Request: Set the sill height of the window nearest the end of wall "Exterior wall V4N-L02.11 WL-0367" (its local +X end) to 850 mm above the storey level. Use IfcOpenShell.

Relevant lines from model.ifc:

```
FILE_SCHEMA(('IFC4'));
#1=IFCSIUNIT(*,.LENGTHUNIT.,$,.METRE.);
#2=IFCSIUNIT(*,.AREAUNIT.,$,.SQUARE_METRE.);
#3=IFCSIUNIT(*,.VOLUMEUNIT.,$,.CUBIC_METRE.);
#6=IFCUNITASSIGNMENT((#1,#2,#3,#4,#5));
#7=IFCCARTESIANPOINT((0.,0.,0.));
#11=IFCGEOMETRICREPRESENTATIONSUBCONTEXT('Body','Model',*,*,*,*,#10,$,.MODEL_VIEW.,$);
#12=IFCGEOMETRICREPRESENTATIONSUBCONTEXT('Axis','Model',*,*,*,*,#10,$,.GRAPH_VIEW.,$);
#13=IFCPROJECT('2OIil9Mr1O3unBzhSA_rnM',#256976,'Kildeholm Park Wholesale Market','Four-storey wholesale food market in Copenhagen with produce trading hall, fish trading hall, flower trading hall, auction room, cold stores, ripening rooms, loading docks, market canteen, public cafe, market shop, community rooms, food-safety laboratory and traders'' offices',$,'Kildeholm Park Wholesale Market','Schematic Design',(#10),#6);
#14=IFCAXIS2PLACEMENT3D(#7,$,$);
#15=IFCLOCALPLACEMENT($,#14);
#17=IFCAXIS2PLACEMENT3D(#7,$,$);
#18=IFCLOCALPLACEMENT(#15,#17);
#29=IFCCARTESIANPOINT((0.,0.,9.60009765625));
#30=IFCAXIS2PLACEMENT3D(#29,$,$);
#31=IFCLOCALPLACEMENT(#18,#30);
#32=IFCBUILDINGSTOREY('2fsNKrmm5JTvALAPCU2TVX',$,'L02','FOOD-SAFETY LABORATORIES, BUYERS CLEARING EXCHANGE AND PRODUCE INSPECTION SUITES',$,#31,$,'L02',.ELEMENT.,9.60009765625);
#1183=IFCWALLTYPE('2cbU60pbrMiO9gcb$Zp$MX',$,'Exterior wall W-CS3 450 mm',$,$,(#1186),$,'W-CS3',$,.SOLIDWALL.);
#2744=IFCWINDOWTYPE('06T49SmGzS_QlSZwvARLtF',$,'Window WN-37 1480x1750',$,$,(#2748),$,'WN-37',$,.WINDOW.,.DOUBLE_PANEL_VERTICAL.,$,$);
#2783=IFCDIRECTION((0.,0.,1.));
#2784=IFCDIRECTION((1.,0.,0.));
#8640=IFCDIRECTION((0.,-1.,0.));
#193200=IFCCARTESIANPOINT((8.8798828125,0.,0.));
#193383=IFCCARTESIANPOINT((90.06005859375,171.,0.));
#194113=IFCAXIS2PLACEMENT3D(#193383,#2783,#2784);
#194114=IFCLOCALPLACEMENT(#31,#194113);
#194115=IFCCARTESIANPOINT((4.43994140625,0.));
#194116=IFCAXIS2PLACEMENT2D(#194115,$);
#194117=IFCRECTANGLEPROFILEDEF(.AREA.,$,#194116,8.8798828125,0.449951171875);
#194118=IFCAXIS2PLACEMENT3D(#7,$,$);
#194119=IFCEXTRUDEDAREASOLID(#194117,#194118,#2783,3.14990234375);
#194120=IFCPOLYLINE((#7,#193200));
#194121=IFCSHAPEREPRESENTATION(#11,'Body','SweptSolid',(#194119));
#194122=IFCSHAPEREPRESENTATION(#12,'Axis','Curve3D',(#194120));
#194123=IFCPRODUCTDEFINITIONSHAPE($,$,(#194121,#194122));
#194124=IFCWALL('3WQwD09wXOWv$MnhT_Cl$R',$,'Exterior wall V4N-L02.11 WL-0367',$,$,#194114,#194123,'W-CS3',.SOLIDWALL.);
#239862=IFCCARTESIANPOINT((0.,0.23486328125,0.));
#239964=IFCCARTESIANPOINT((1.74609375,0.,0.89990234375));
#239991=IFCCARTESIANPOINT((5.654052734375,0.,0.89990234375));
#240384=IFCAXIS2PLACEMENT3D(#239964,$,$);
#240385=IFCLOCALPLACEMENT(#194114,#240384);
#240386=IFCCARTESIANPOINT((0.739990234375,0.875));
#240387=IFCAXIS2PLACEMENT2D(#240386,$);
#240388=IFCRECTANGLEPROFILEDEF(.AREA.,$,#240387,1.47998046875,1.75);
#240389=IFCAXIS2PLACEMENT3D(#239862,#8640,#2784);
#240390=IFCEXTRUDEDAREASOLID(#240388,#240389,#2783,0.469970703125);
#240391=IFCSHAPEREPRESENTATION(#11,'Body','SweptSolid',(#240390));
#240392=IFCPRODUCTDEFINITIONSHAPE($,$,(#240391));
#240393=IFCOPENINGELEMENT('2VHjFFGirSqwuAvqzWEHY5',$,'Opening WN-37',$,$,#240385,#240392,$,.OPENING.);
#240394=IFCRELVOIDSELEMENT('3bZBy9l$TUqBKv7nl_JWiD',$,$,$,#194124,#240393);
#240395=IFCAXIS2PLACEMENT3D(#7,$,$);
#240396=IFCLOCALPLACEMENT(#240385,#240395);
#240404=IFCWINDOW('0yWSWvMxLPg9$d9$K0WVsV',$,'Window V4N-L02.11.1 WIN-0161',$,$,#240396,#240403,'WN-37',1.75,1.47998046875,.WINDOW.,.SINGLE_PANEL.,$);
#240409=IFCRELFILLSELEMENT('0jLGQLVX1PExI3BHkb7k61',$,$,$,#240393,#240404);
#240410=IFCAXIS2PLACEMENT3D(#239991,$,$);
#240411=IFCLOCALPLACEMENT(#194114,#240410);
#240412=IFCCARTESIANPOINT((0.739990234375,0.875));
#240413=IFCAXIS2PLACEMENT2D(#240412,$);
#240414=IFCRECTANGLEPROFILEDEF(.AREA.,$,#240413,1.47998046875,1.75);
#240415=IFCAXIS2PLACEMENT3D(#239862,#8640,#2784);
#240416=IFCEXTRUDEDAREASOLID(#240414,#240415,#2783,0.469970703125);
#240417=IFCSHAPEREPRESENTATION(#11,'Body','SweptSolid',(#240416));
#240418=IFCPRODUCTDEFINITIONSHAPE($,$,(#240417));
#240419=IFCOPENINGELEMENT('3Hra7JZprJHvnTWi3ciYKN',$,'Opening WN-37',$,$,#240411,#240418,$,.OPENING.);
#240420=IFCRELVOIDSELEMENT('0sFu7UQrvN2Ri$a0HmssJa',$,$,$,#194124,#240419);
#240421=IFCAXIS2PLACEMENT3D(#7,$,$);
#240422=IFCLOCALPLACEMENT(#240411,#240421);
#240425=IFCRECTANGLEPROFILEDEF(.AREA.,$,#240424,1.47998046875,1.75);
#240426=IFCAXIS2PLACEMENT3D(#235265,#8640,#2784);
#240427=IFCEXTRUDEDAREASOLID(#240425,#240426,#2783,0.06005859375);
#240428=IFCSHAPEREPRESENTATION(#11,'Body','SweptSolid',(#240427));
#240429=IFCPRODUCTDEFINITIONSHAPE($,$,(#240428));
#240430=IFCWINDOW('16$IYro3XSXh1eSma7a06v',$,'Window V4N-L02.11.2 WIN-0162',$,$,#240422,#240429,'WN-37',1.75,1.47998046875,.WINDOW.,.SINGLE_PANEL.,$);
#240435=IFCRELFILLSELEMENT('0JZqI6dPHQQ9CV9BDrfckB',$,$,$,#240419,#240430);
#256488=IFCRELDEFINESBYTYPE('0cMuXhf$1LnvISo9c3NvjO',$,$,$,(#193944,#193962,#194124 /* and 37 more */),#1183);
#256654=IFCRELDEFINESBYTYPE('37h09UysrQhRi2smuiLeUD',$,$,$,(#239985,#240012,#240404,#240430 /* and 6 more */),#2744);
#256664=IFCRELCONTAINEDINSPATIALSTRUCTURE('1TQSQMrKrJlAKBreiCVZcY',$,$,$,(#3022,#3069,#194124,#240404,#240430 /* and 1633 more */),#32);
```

```python
import numpy as np
import ifcopenshell
import ifcopenshell.api.geometry
import ifcopenshell.geom
import ifcopenshell.util.element
import ifcopenshell.util.placement
import ifcopenshell.util.shape
import ifcopenshell.util.unit

model = ifcopenshell.open("model.ifc")
unit_scale = ifcopenshell.util.unit.calculate_unit_scale(model)

window = model.by_guid("16$IYro3XSXh1eSma7a06v")
opening = window.FillsVoids[0].RelatingOpeningElement
storey = ifcopenshell.util.element.get_container(window, ifc_class="IfcBuildingStorey")
level = ifcopenshell.util.placement.get_local_placement(storey.ObjectPlacement)[2, 3]

# The opening's origin need not be at the sill, so measure its lowest point.
shape = ifcopenshell.geom.create_shape(ifcopenshell.geom.settings(), opening)
bottom = ifcopenshell.util.shape.get_shape_bottom_elevation(shape, shape.geometry) / unit_scale
dz = level + 0.85 - bottom

shift = np.array([0.0, 0.0, dz])
# The window is placed relative to its opening, so it follows when the opening moves.
matrix = ifcopenshell.util.placement.get_local_placement(opening.ObjectPlacement)
matrix[:3, 3] += shift
ifcopenshell.api.geometry.edit_object_placement(
    model, product=opening, matrix=matrix, is_si=False, should_transform_children=True
)

print(f"moved by {dz * unit_scale:+.3f} m")

model.write("model_v2.ifc")
```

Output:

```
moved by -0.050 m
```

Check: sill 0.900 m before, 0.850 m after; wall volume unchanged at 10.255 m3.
